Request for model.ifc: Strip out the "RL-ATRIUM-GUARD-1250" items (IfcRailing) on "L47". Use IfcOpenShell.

First a look at what the model holds.

```python
import ifcopenshell
import ifcopenshell.util.element

model = ifcopenshell.open("model.ifc")
print(model.schema)
storey = next(s for s in model.by_type("IfcBuildingStorey") if s.Name == "L47")
railings = [e for e in ifcopenshell.util.element.get_decomposition(storey) if e.is_a("IfcRailing")]
seen = {}
for e in railings:
    element_type = ifcopenshell.util.element.get_type(e)
    name = element_type.Name if element_type not in (None, e) else None
    seen[name] = seen.get(name, 0) + 1
for name, count in sorted(seen.items(), key=str):
    print(count, "x", name)
```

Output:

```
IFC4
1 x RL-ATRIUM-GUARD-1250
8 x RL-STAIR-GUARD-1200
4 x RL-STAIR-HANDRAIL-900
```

```python
import ifcopenshell
import ifcopenshell.api.root
import ifcopenshell.util.element

model = ifcopenshell.open("model.ifc")

storey = next(s for s in model.by_type("IfcBuildingStorey") if s.Name == "L47")
railings = [e for e in ifcopenshell.util.element.get_decomposition(storey) if e.is_a("IfcRailing")]
targets = [e for e in railings if (t := ifcopenshell.util.element.get_type(e)) not in (None, e) and t.Name == "RL-ATRIUM-GUARD-1250"]

for e in targets:
    ifcopenshell.api.root.remove_product(model, product=e)
print(len(targets), "removed")

model.write("model_rev.ifc")
```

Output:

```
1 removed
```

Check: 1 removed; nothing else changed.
